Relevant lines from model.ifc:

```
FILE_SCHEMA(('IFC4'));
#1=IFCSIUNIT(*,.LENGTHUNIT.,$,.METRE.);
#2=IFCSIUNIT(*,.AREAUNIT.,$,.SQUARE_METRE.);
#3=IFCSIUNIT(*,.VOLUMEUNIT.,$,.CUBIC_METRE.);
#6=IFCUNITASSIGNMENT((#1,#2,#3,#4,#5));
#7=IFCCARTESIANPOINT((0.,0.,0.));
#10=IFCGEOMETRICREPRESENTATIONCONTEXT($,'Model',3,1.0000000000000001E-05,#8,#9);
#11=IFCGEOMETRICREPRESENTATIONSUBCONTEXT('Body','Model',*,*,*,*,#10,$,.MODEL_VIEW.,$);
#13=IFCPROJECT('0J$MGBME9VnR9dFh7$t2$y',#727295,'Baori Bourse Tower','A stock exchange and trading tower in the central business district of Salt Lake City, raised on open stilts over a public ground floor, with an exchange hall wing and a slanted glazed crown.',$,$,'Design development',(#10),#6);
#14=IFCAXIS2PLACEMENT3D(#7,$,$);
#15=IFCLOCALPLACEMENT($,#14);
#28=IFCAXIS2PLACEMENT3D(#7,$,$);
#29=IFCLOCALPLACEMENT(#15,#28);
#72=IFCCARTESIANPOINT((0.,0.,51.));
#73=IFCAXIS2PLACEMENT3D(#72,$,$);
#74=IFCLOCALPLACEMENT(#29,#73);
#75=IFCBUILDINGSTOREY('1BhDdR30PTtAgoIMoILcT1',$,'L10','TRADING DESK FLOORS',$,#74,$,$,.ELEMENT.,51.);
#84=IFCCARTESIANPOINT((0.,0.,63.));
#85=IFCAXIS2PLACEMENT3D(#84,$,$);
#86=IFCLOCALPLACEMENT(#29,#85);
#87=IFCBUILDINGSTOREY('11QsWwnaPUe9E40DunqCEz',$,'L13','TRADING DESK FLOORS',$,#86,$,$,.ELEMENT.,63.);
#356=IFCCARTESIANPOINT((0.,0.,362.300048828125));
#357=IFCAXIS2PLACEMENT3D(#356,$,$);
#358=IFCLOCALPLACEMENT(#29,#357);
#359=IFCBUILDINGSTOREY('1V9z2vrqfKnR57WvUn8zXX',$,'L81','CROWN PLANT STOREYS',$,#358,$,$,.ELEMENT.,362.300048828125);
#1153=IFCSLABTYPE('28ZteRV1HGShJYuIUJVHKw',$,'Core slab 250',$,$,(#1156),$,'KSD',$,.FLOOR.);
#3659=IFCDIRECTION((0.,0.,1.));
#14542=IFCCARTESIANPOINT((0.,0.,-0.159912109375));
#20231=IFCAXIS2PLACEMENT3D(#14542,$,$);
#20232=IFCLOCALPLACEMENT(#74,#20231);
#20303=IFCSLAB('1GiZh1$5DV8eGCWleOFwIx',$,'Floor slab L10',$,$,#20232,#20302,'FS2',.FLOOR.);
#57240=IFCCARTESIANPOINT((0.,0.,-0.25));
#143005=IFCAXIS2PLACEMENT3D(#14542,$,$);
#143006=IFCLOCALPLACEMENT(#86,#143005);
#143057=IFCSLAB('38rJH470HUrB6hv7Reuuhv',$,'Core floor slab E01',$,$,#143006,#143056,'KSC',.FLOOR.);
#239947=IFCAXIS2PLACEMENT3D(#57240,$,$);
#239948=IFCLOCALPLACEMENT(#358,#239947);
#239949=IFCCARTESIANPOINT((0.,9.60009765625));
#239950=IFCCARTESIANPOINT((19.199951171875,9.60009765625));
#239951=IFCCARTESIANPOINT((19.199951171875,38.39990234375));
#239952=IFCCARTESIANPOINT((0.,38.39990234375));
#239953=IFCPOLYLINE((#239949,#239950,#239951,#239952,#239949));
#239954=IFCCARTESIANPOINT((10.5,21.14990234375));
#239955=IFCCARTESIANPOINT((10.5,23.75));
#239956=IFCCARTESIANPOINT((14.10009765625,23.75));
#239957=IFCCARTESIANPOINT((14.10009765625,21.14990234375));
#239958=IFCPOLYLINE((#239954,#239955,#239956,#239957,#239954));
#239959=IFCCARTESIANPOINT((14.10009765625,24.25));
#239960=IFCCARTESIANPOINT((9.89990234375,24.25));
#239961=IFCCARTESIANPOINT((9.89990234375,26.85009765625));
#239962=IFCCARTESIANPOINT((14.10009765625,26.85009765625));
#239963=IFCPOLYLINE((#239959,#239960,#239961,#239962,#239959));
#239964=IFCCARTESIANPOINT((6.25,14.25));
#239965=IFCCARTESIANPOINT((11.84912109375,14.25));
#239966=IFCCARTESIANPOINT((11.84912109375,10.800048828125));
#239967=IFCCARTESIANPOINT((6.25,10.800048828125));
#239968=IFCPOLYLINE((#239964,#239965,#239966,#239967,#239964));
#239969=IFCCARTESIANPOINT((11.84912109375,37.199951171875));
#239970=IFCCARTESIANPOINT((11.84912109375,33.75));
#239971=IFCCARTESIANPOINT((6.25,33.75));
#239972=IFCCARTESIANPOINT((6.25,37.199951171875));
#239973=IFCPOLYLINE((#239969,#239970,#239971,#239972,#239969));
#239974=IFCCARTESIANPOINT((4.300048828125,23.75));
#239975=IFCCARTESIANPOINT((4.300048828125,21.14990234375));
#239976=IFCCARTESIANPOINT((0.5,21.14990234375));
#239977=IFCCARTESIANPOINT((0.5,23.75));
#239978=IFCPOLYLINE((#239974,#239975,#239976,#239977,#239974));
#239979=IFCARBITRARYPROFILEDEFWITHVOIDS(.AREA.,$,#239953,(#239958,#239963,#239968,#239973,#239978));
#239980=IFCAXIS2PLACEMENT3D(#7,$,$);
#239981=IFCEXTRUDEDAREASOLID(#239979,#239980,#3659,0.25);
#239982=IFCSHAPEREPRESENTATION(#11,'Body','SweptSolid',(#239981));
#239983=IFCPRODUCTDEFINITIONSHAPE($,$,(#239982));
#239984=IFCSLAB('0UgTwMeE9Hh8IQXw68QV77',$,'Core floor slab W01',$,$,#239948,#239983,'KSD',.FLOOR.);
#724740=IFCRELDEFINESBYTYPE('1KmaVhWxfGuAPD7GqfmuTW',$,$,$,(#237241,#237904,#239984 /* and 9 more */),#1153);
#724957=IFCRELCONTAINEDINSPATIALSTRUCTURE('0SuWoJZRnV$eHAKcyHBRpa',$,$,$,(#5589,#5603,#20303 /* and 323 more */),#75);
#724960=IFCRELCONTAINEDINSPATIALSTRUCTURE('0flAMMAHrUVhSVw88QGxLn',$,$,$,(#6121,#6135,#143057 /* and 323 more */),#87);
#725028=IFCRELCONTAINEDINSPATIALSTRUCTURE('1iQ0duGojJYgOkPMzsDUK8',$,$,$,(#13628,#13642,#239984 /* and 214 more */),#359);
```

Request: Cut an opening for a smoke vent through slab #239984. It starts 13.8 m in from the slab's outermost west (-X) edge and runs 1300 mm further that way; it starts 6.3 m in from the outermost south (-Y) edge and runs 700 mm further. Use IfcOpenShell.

```python
import numpy as np
import ifcopenshell
import ifcopenshell.api.feature
import ifcopenshell.api.geometry
import ifcopenshell.api.root
import ifcopenshell.geom
import ifcopenshell.util.placement
import ifcopenshell.util.representation
import ifcopenshell.util.shape
import ifcopenshell.util.unit

model = ifcopenshell.open("model.ifc")
unit_scale = ifcopenshell.util.unit.calculate_unit_scale(model)
settings = ifcopenshell.geom.settings()


def volume(element):
    """Net volume in cubic metres, openings subtracted."""
    shape = ifcopenshell.geom.create_shape(settings, element)
    return ifcopenshell.util.shape.get_volume(shape.geometry)


slab = model.by_guid("0UgTwMeE9Hh8IQXw68QV77")
before = volume(slab)

# Extent in the slab's own axes, in metres. The edges named are its -X and -Y sides.
slab_shape = ifcopenshell.geom.create_shape(settings, slab)
vertices = ifcopenshell.util.shape.get_vertices(slab_shape.geometry)
x_min, y_min, bottom = vertices.min(axis=0)
top = vertices[:, 2].max()

opening = ifcopenshell.api.root.create_entity(model, ifc_class="IfcOpeningElement", name="Smoke vent opening", predefined_type="OPENING")
context = ifcopenshell.util.representation.get_context(model, "Model", "Body", "MODEL_VIEW")
width, depth = 1.3, 0.7
outline = [(0.0, 0.0), (width, 0.0), (width, depth), (0.0, depth), (0.0, 0.0)]
# Overshoot both faces by 50 mm so the cut is clean.
shape = ifcopenshell.api.geometry.add_slab_representation(
    model, context=context, depth=top - bottom + 0.1, polyline=outline
)
ifcopenshell.api.geometry.assign_representation(model, product=opening, representation=shape)

matrix = ifcopenshell.util.placement.get_local_placement(slab.ObjectPlacement)
matrix[:, 3] = matrix @ np.append(np.array([x_min + 13.8, y_min + 6.3, bottom - 0.05]) / unit_scale, 1.0)
ifcopenshell.api.geometry.edit_object_placement(model, product=opening, matrix=matrix, is_si=False)
ifcopenshell.api.feature.add_feature(model, feature=opening, element=slab)

after = volume(slab)

print(f"slab volume {before:.3f} -> {after:.3f} m3")

model.write("model_rev.ifc")
```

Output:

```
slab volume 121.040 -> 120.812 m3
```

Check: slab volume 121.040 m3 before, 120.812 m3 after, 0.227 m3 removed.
